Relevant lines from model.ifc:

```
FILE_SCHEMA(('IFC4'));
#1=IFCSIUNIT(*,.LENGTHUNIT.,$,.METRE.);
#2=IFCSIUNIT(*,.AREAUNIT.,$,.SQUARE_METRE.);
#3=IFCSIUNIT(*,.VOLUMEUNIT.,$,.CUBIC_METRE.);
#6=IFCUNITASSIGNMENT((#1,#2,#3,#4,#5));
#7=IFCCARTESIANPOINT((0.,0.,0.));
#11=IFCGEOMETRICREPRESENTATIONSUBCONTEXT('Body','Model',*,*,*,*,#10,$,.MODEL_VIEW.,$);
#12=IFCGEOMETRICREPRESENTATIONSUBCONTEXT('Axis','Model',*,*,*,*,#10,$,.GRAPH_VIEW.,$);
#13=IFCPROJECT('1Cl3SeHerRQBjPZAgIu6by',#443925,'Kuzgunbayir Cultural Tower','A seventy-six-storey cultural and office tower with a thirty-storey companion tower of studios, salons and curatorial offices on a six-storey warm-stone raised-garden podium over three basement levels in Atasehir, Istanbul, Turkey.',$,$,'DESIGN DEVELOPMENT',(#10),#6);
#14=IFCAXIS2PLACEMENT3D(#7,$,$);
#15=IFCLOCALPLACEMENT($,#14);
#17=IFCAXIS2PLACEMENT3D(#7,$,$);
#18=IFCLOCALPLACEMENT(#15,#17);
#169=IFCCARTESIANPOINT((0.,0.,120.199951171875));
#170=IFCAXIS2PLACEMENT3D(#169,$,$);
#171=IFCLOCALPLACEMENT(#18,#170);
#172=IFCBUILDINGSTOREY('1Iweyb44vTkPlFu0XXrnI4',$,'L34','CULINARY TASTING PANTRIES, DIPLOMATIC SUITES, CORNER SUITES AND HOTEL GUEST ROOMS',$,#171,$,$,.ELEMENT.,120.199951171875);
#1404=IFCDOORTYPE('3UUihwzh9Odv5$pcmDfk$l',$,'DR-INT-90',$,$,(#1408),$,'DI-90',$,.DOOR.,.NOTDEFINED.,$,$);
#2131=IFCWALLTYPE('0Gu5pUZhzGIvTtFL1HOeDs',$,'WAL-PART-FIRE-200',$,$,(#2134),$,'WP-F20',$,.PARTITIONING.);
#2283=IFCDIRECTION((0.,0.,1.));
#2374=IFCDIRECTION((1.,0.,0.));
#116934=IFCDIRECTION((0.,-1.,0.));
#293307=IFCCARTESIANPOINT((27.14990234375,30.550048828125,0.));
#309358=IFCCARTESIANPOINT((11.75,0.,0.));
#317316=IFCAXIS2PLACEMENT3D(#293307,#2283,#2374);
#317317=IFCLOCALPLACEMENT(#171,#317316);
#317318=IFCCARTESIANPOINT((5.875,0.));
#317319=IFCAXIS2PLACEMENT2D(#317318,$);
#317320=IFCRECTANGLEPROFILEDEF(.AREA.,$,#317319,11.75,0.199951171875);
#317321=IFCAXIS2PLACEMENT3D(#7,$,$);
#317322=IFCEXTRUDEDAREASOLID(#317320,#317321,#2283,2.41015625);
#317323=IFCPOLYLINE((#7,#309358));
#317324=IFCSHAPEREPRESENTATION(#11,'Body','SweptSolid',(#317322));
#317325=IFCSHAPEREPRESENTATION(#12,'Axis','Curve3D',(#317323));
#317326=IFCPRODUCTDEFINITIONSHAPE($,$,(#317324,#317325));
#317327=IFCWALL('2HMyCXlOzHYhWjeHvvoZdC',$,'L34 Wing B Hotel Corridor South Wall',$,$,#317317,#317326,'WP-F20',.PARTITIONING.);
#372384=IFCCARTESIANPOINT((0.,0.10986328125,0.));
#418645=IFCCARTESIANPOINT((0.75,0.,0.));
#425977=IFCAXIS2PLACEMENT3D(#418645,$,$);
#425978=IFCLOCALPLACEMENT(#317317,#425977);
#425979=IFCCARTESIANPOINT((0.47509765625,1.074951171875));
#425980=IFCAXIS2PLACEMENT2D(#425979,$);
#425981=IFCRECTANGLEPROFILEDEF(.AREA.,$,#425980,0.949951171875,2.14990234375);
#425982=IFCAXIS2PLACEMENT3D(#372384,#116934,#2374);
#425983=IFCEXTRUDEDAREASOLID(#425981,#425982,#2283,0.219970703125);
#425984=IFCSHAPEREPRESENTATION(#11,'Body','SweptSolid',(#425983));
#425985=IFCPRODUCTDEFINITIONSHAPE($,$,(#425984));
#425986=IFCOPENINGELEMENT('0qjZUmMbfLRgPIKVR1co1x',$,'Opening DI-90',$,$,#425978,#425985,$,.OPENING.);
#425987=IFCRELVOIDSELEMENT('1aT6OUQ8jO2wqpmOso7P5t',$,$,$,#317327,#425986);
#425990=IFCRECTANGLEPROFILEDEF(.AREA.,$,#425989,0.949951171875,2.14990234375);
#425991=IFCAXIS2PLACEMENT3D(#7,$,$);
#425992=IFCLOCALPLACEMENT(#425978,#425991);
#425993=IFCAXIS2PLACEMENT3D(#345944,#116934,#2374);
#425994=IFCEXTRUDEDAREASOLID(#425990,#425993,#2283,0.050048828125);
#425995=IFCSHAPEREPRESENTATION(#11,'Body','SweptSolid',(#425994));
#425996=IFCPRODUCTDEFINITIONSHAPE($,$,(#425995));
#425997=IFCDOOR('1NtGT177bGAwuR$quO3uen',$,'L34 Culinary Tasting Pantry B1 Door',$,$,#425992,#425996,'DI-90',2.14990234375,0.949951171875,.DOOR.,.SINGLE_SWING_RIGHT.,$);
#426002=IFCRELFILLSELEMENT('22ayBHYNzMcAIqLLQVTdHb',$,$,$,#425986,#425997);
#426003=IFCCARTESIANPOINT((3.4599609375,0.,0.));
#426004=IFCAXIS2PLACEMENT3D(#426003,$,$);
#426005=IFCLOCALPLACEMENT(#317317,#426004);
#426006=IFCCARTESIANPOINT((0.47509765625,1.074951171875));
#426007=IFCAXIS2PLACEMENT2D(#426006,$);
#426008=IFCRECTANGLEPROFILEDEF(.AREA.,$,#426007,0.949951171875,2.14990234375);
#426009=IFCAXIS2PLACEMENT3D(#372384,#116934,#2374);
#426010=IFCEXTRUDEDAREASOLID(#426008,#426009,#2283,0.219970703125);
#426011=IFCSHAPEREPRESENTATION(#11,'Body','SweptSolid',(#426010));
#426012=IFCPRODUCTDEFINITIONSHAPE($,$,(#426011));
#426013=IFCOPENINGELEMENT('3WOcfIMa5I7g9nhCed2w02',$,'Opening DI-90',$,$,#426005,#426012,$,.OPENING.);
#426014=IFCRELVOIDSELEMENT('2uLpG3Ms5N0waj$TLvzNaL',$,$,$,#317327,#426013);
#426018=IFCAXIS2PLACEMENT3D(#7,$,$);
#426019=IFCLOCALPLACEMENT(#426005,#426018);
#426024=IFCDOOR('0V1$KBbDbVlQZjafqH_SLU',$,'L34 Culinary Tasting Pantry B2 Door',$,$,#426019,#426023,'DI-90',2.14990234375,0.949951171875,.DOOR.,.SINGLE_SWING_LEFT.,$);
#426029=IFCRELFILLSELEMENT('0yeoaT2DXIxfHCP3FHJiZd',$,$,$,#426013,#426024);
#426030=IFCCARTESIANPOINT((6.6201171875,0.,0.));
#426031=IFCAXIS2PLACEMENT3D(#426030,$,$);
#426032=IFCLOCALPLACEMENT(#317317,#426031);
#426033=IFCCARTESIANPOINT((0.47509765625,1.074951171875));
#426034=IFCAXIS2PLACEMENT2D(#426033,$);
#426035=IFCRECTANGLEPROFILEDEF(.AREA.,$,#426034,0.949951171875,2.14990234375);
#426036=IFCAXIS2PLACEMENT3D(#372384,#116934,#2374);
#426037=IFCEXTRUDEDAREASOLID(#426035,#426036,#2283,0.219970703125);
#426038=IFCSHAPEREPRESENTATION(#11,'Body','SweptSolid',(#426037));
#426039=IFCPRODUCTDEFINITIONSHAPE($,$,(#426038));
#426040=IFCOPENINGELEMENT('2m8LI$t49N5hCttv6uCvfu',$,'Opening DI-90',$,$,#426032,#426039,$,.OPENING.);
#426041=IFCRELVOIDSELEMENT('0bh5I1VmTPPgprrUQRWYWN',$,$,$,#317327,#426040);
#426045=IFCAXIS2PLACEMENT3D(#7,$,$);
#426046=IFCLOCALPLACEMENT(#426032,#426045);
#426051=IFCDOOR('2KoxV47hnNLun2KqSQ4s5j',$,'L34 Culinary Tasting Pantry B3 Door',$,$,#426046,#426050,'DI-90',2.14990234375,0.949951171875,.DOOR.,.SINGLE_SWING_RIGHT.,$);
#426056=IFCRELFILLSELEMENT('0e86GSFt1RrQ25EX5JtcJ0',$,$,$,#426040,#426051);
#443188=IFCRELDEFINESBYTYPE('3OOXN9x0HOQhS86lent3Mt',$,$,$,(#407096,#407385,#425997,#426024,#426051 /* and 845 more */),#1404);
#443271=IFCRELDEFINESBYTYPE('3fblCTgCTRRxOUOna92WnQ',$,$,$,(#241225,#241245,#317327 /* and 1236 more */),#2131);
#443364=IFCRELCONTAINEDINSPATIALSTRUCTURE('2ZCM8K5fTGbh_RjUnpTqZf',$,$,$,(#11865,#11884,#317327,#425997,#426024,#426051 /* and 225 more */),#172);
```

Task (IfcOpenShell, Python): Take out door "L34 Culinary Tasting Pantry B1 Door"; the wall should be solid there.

```python
import ifcopenshell
import ifcopenshell.api.feature
import ifcopenshell.api.root
import ifcopenshell.geom
import ifcopenshell.util.shape

model = ifcopenshell.open("model.ifc")
settings = ifcopenshell.geom.settings()


def volume(element):
    """Net volume in cubic metres, openings subtracted."""
    shape = ifcopenshell.geom.create_shape(settings, element)
    return ifcopenshell.util.shape.get_volume(shape.geometry)


door = model.by_id(425997)
opening = door.FillsVoids[0].RelatingOpeningElement
wall = opening.VoidsElements[0].RelatingBuildingElement
before = volume(wall)

ifcopenshell.api.root.remove_product(model, product=door)
ifcopenshell.api.feature.remove_feature(model, feature=opening)

after = volume(wall)

print(f"wall volume {before:.3f} -> {after:.3f} m3")

model.write("model_v2.ifc")
```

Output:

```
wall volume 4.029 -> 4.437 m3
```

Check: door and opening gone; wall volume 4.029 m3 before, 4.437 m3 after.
